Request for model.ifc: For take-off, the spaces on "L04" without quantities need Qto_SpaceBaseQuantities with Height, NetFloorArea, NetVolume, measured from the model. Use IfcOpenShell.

First a look at what the model holds.

```python
import ifcopenshell
import ifcopenshell.util.element
import ifcopenshell.util.unit

model = ifcopenshell.open("model.ifc")
print(model.schema)
for unit_type in ("LENGTHUNIT", "AREAUNIT", "VOLUMEUNIT"):
    print(unit_type, ifcopenshell.util.unit.calculate_unit_scale(model, unit_type))
storey = next(s for s in model.by_type("IfcBuildingStorey") if s.Name == "L04")
spaces = [e for e in ifcopenshell.util.element.get_decomposition(storey) if e.is_a("IfcSpace")]
for e in sorted(spaces, key=lambda e: e.id()):
    print(e.id(), e.is_a(), e.Name, list(ifcopenshell.util.element.get_psets(e, qtos_only=True)), sep=" | ")
```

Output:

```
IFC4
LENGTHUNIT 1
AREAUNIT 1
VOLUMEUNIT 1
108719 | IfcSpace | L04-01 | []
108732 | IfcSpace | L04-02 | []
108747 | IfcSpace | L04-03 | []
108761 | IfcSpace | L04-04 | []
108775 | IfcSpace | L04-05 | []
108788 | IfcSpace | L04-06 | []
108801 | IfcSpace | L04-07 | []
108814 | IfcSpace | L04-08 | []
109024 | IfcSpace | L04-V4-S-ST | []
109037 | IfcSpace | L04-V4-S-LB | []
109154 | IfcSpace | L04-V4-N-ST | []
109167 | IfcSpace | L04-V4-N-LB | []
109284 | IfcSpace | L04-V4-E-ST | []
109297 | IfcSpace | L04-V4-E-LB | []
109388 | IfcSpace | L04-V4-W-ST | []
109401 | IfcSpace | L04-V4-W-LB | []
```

```python
import ifcopenshell
import ifcopenshell.api.pset
import ifcopenshell.geom
import ifcopenshell.util.element
import ifcopenshell.util.shape
import ifcopenshell.util.unit

model = ifcopenshell.open("model.ifc")
unit_scale = ifcopenshell.util.unit.calculate_unit_scale(model)
area_scale = ifcopenshell.util.unit.calculate_unit_scale(model, "AREAUNIT")
volume_scale = ifcopenshell.util.unit.calculate_unit_scale(model, "VOLUMEUNIT")
settings = ifcopenshell.geom.settings()

storey = next(s for s in model.by_type("IfcBuildingStorey") if s.Name == "L04")
spaces = [e for e in ifcopenshell.util.element.get_decomposition(storey) if e.is_a("IfcSpace")]

for e in sorted(spaces, key=lambda e: e.id()):
    if ifcopenshell.util.element.get_psets(e, qtos_only=True, should_inherit=False):
        continue
    # Geometry comes back in metres, in the element's own axes.
    shape = ifcopenshell.geom.create_shape(settings, e)
    values = {
        "Height": ifcopenshell.util.shape.get_z(shape.geometry) / unit_scale,
        "NetFloorArea": ifcopenshell.util.shape.get_footprint_area(shape.geometry) / area_scale,
        "NetVolume": ifcopenshell.util.shape.get_volume(shape.geometry) / volume_scale,
    }
    qto = ifcopenshell.api.pset.add_qto(model, product=e, name="Qto_SpaceBaseQuantities")
    ifcopenshell.api.pset.edit_qto(model, qto=qto, properties=values)
    print(e.id(), {k: round(v, 3) for k, v in values.items()})

model.write("model_v2.ifc")
```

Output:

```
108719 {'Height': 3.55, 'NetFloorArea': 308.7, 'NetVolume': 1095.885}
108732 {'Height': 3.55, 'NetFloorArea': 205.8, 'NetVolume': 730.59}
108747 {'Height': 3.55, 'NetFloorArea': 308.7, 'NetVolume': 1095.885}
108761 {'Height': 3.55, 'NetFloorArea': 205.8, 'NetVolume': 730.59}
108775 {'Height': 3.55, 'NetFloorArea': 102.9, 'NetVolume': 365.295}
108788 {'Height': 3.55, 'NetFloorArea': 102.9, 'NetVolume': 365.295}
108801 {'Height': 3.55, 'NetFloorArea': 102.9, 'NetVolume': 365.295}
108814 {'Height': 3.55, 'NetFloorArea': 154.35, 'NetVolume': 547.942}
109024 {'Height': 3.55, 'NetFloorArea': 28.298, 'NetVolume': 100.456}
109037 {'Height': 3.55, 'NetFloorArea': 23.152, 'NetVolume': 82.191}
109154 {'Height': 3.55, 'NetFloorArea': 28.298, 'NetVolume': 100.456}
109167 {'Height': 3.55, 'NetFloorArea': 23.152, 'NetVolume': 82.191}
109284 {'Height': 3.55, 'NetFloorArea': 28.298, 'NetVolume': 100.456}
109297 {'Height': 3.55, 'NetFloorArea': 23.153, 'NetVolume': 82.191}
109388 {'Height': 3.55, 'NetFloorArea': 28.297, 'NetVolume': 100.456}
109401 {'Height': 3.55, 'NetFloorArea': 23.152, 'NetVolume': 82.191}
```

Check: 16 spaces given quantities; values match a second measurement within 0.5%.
